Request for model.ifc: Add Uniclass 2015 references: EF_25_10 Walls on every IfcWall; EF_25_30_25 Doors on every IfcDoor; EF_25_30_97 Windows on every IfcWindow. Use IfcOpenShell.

First a look at what the model holds.

```python
import ifcopenshell

model = ifcopenshell.open("model.ifc")
print(model.schema)
print("classifications:", [c.Name for c in model.by_type("IfcClassification")])
for ifc_class in ("IfcDoor", "IfcRoof", "IfcStair", "IfcWall", "IfcWindow"):
    print(ifc_class, len(model.by_type(ifc_class)))
```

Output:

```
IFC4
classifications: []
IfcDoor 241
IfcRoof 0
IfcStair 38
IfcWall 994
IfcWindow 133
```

```python
import ifcopenshell
import ifcopenshell.api.classification

model = ifcopenshell.open("model.ifc")

system = ifcopenshell.api.classification.add_classification(model, classification="Uniclass 2015")

codes = {
    "IfcWall": ("EF_25_10", "Walls"),
    "IfcDoor": ("EF_25_30_25", "Doors"),
    "IfcWindow": ("EF_25_30_97", "Windows"),
}
for ifc_class, (code, name) in codes.items():
    products = model.by_type(ifc_class)
    ifcopenshell.api.classification.add_reference(
        model, products=products, classification=system, identification=code, name=name
    )
    print(code, len(products))

model.write("model_v2.ifc")
```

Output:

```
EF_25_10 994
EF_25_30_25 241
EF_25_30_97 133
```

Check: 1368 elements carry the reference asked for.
